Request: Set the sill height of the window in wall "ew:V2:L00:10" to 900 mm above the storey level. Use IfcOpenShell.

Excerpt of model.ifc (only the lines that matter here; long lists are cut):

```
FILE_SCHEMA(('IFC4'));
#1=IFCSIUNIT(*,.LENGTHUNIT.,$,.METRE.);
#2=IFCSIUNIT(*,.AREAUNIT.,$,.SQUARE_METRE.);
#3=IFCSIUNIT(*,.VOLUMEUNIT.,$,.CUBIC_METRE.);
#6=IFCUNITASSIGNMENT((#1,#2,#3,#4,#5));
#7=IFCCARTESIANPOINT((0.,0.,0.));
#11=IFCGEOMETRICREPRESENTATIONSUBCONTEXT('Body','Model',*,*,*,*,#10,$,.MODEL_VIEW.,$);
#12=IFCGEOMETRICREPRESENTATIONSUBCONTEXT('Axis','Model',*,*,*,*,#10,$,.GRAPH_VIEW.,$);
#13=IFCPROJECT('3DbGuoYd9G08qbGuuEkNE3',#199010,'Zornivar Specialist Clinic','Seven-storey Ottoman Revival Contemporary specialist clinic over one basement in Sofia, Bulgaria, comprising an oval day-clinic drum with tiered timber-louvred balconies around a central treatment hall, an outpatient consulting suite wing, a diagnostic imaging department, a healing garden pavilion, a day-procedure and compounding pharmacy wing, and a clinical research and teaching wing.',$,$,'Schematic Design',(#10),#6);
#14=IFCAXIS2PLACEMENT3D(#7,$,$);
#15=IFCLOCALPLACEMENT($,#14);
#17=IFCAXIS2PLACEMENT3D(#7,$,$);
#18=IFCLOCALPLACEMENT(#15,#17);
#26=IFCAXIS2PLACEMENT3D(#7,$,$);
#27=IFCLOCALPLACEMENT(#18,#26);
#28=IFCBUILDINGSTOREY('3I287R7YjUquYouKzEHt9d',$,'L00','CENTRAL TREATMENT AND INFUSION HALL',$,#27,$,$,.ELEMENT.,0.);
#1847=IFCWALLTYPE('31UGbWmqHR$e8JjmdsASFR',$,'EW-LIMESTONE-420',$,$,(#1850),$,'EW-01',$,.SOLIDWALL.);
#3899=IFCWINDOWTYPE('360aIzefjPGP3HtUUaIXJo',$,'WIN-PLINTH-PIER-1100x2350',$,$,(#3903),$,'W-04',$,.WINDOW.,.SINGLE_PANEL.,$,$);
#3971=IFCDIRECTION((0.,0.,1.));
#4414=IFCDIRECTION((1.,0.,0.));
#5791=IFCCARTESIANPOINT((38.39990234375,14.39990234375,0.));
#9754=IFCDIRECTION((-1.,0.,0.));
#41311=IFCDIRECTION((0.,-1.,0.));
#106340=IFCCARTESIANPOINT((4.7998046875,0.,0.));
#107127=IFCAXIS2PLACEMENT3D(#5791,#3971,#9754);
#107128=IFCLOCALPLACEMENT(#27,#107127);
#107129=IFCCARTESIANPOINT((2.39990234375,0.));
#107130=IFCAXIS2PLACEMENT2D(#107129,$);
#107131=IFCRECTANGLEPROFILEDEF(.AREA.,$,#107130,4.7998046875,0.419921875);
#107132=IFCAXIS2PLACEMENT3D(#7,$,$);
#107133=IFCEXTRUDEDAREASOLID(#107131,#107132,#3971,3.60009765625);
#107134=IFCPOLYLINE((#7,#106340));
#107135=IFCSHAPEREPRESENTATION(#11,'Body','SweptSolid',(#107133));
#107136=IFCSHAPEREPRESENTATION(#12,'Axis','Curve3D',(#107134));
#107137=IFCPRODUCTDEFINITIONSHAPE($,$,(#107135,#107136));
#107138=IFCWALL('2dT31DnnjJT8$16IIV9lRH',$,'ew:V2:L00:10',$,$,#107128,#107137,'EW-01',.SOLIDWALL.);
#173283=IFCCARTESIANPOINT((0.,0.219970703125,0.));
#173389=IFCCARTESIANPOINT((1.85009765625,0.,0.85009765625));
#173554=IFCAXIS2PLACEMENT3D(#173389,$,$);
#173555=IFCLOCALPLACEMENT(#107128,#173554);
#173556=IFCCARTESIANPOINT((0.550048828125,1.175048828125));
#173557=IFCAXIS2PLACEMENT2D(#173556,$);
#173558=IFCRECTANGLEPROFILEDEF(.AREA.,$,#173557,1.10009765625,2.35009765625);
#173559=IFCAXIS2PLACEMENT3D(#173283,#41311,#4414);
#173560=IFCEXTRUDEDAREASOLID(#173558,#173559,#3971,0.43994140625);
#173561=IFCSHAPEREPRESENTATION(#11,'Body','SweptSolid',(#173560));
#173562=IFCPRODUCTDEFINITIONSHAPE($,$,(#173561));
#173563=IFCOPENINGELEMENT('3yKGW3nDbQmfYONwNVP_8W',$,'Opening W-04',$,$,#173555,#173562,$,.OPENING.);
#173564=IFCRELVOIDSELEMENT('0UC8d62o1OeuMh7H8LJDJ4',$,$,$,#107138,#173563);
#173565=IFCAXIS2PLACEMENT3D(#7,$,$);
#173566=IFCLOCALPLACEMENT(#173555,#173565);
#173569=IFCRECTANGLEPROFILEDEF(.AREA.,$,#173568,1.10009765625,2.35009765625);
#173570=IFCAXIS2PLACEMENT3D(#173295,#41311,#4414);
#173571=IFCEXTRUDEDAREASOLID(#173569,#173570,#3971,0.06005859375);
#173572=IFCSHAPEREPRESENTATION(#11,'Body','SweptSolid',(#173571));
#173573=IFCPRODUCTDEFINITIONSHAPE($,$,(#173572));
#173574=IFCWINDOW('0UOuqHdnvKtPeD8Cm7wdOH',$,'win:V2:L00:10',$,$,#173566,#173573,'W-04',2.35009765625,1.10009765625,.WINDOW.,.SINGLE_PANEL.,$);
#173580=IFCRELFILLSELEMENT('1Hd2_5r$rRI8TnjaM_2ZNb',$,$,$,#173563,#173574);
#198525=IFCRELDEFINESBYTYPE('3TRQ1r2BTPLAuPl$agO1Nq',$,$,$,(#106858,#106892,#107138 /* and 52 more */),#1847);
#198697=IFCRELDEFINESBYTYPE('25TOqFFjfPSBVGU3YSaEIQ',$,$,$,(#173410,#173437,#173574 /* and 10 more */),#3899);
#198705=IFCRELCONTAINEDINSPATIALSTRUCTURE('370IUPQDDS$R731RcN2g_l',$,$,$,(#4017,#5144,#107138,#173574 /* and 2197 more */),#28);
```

```python
import numpy as np
import ifcopenshell
import ifcopenshell.api.geometry
import ifcopenshell.geom
import ifcopenshell.util.element
import ifcopenshell.util.placement
import ifcopenshell.util.shape
import ifcopenshell.util.unit

model = ifcopenshell.open("model.ifc")
unit_scale = ifcopenshell.util.unit.calculate_unit_scale(model)

window = model.by_guid("0UOuqHdnvKtPeD8Cm7wdOH")
opening = window.FillsVoids[0].RelatingOpeningElement
storey = ifcopenshell.util.element.get_container(window, ifc_class="IfcBuildingStorey")
level = ifcopenshell.util.placement.get_local_placement(storey.ObjectPlacement)[2, 3]

# The opening's origin need not be at the sill, so measure its lowest point.
shape = ifcopenshell.geom.create_shape(ifcopenshell.geom.settings(), opening)
bottom = ifcopenshell.util.shape.get_shape_bottom_elevation(shape, shape.geometry) / unit_scale
dz = level + 0.9 / unit_scale - bottom

shift = np.array([0.0, 0.0, dz])
# The window is placed relative to its opening, so it follows when the opening moves.
matrix = ifcopenshell.util.placement.get_local_placement(opening.ObjectPlacement)
matrix[:3, 3] += shift
ifcopenshell.api.geometry.edit_object_placement(
    model, product=opening, matrix=matrix, is_si=False, should_transform_children=True
)

print(f"moved by {dz * unit_scale:+.3f} m")

model.write("model-out.ifc")
```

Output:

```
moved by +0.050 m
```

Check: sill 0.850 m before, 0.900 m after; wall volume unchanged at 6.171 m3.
